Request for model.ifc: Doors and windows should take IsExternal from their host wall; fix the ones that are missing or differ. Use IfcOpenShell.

First a look at what the model holds.

```python
import ifcopenshell
import ifcopenshell.util.element

model = ifcopenshell.open("model.ifc")
print(model.schema)
seen = {}
for e in model.by_type("IfcDoor") + model.by_type("IfcWindow"):
    if not e.FillsVoids:
        continue
    host = e.FillsVoids[0].RelatingOpeningElement.VoidsElements[0].RelatingBuildingElement
    own = ifcopenshell.util.element.get_pset(e, f"Pset_{e.is_a()[3:].removesuffix('StandardCase')}Common", "IsExternal")
    wall = ifcopenshell.util.element.get_pset(host, "Pset_WallCommon", "IsExternal")
    seen[e.is_a(), own, wall] = seen.get((e.is_a(), own, wall), 0) + 1
for (cls, own, wall), count in sorted(seen.items(), key=str):
    print(count, cls, "IsExternal:", own, "| host wall:", wall)
```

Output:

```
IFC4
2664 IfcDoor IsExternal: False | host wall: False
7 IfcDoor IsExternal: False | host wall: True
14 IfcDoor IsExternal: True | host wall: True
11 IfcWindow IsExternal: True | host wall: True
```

```python
import ifcopenshell
import ifcopenshell.api.pset
import ifcopenshell.util.element

model = ifcopenshell.open("model.ifc")

count = 0
for ifc_class, pset_name in (("IfcDoor", "Pset_DoorCommon"), ("IfcWindow", "Pset_WindowCommon")):
    for e in model.by_type(ifc_class):
        if not e.FillsVoids:
            continue
        host = e.FillsVoids[0].RelatingOpeningElement.VoidsElements[0].RelatingBuildingElement
        external = ifcopenshell.util.element.get_pset(host, "Pset_WallCommon", "IsExternal")
        if external is None or ifcopenshell.util.element.get_pset(e, pset_name, "IsExternal") == external:
            continue
        pset = ifcopenshell.api.pset.add_pset(model, product=e, name=pset_name)
        ifcopenshell.api.pset.edit_pset(model, pset=pset, properties={"IsExternal": external})
        count += 1

print(count, "updated")

model.write("model_rev.ifc")
```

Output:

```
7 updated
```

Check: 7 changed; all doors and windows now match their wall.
